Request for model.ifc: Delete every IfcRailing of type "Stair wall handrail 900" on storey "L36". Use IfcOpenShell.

First a look at what the model holds.

```python
import ifcopenshell
import ifcopenshell.util.element

model = ifcopenshell.open("model.ifc")
print(model.schema)
storey = next(s for s in model.by_type("IfcBuildingStorey") if s.Name == "L36")
railings = [e for e in ifcopenshell.util.element.get_decomposition(storey) if e.is_a("IfcRailing")]
seen = {}
for e in railings:
    element_type = ifcopenshell.util.element.get_type(e)
    name = element_type.Name if element_type not in (None, e) else None
    seen[name] = seen.get(name, 0) + 1
for name, count in sorted(seen.items(), key=str):
    print(count, "x", name)
```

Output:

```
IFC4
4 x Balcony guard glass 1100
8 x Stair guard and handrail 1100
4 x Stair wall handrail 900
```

```python
import ifcopenshell
import ifcopenshell.api.root
import ifcopenshell.util.element

model = ifcopenshell.open("model.ifc")

storey = next(s for s in model.by_type("IfcBuildingStorey") if s.Name == "L36")
railings = [e for e in ifcopenshell.util.element.get_decomposition(storey) if e.is_a("IfcRailing")]
targets = [e for e in railings if (t := ifcopenshell.util.element.get_type(e)) not in (None, e) and t.Name == "Stair wall handrail 900"]

for e in targets:
    ifcopenshell.api.root.remove_product(model, product=e)
print(len(targets), "removed")

model.write("model_rev.ifc")
```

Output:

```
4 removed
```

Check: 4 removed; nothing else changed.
